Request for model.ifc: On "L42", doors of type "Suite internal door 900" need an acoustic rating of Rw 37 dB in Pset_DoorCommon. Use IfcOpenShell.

First a look at what the model holds.

```python
import ifcopenshell
import ifcopenshell.util.element

model = ifcopenshell.open("model.ifc")
print(model.schema)
storey = next(s for s in model.by_type("IfcBuildingStorey") if s.Name == "L42")
doors = [e for e in ifcopenshell.util.element.get_decomposition(storey) if e.is_a("IfcDoor")]
seen = {}
for e in doors:
    element_type = ifcopenshell.util.element.get_type(e)
    key = (element_type.Name if element_type != e and element_type else None, ifcopenshell.util.element.get_pset(e, "Pset_DoorCommon", "AcousticRating"))
    seen[key] = seen.get(key, 0) + 1
for (name, value), count in sorted(seen.items(), key=str):
    print(count, "x", name, "|", value)
```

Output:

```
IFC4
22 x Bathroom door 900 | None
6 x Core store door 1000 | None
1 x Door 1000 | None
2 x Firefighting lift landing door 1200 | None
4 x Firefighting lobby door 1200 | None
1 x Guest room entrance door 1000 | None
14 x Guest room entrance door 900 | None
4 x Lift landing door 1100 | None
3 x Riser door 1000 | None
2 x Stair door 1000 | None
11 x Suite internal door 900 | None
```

```python
import ifcopenshell
import ifcopenshell.api.pset
import ifcopenshell.util.element

model = ifcopenshell.open("model.ifc")

storey = next(s for s in model.by_type("IfcBuildingStorey") if s.Name == "L42")
doors = [e for e in ifcopenshell.util.element.get_decomposition(storey) if e.is_a("IfcDoor")]

count = 0
for e in doors:
    element_type = ifcopenshell.util.element.get_type(e)
    if element_type in (None, e) or element_type.Name != "Suite internal door 900":
        continue
    # add_pset returns the element's existing set when there is one.
    pset = ifcopenshell.api.pset.add_pset(model, product=e, name="Pset_DoorCommon")
    ifcopenshell.api.pset.edit_pset(model, pset=pset, properties={"AcousticRating": "Rw 37 dB"})
    count += 1

print(count, "doors updated")

model.write("model-out.ifc")
```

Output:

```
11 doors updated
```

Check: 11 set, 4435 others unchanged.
